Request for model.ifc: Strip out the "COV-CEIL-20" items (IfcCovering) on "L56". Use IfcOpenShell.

First a look at what the model holds.

```python
import ifcopenshell
import ifcopenshell.util.element

model = ifcopenshell.open("model.ifc")
print(model.schema)
storey = next(s for s in model.by_type("IfcBuildingStorey") if s.Name == "L56")
coverings = [e for e in ifcopenshell.util.element.get_decomposition(storey) if e.is_a("IfcCovering")]
seen = {}
for e in coverings:
    element_type = ifcopenshell.util.element.get_type(e)
    name = element_type.Name if element_type not in (None, e) else None
    seen[name] = seen.get(name, 0) + 1
for name, count in sorted(seen.items(), key=str):
    print(count, "x", name)
```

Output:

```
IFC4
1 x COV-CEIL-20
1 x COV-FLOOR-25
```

```python
import ifcopenshell
import ifcopenshell.api.root
import ifcopenshell.util.element

model = ifcopenshell.open("model.ifc")

storey = next(s for s in model.by_type("IfcBuildingStorey") if s.Name == "L56")
coverings = [e for e in ifcopenshell.util.element.get_decomposition(storey) if e.is_a("IfcCovering")]
targets = [e for e in coverings if (t := ifcopenshell.util.element.get_type(e)) not in (None, e) and t.Name == "COV-CEIL-20"]

for e in targets:
    ifcopenshell.api.root.remove_product(model, product=e)
print(len(targets), "removed")

model.write("model_rev.ifc")
```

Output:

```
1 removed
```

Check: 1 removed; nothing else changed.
